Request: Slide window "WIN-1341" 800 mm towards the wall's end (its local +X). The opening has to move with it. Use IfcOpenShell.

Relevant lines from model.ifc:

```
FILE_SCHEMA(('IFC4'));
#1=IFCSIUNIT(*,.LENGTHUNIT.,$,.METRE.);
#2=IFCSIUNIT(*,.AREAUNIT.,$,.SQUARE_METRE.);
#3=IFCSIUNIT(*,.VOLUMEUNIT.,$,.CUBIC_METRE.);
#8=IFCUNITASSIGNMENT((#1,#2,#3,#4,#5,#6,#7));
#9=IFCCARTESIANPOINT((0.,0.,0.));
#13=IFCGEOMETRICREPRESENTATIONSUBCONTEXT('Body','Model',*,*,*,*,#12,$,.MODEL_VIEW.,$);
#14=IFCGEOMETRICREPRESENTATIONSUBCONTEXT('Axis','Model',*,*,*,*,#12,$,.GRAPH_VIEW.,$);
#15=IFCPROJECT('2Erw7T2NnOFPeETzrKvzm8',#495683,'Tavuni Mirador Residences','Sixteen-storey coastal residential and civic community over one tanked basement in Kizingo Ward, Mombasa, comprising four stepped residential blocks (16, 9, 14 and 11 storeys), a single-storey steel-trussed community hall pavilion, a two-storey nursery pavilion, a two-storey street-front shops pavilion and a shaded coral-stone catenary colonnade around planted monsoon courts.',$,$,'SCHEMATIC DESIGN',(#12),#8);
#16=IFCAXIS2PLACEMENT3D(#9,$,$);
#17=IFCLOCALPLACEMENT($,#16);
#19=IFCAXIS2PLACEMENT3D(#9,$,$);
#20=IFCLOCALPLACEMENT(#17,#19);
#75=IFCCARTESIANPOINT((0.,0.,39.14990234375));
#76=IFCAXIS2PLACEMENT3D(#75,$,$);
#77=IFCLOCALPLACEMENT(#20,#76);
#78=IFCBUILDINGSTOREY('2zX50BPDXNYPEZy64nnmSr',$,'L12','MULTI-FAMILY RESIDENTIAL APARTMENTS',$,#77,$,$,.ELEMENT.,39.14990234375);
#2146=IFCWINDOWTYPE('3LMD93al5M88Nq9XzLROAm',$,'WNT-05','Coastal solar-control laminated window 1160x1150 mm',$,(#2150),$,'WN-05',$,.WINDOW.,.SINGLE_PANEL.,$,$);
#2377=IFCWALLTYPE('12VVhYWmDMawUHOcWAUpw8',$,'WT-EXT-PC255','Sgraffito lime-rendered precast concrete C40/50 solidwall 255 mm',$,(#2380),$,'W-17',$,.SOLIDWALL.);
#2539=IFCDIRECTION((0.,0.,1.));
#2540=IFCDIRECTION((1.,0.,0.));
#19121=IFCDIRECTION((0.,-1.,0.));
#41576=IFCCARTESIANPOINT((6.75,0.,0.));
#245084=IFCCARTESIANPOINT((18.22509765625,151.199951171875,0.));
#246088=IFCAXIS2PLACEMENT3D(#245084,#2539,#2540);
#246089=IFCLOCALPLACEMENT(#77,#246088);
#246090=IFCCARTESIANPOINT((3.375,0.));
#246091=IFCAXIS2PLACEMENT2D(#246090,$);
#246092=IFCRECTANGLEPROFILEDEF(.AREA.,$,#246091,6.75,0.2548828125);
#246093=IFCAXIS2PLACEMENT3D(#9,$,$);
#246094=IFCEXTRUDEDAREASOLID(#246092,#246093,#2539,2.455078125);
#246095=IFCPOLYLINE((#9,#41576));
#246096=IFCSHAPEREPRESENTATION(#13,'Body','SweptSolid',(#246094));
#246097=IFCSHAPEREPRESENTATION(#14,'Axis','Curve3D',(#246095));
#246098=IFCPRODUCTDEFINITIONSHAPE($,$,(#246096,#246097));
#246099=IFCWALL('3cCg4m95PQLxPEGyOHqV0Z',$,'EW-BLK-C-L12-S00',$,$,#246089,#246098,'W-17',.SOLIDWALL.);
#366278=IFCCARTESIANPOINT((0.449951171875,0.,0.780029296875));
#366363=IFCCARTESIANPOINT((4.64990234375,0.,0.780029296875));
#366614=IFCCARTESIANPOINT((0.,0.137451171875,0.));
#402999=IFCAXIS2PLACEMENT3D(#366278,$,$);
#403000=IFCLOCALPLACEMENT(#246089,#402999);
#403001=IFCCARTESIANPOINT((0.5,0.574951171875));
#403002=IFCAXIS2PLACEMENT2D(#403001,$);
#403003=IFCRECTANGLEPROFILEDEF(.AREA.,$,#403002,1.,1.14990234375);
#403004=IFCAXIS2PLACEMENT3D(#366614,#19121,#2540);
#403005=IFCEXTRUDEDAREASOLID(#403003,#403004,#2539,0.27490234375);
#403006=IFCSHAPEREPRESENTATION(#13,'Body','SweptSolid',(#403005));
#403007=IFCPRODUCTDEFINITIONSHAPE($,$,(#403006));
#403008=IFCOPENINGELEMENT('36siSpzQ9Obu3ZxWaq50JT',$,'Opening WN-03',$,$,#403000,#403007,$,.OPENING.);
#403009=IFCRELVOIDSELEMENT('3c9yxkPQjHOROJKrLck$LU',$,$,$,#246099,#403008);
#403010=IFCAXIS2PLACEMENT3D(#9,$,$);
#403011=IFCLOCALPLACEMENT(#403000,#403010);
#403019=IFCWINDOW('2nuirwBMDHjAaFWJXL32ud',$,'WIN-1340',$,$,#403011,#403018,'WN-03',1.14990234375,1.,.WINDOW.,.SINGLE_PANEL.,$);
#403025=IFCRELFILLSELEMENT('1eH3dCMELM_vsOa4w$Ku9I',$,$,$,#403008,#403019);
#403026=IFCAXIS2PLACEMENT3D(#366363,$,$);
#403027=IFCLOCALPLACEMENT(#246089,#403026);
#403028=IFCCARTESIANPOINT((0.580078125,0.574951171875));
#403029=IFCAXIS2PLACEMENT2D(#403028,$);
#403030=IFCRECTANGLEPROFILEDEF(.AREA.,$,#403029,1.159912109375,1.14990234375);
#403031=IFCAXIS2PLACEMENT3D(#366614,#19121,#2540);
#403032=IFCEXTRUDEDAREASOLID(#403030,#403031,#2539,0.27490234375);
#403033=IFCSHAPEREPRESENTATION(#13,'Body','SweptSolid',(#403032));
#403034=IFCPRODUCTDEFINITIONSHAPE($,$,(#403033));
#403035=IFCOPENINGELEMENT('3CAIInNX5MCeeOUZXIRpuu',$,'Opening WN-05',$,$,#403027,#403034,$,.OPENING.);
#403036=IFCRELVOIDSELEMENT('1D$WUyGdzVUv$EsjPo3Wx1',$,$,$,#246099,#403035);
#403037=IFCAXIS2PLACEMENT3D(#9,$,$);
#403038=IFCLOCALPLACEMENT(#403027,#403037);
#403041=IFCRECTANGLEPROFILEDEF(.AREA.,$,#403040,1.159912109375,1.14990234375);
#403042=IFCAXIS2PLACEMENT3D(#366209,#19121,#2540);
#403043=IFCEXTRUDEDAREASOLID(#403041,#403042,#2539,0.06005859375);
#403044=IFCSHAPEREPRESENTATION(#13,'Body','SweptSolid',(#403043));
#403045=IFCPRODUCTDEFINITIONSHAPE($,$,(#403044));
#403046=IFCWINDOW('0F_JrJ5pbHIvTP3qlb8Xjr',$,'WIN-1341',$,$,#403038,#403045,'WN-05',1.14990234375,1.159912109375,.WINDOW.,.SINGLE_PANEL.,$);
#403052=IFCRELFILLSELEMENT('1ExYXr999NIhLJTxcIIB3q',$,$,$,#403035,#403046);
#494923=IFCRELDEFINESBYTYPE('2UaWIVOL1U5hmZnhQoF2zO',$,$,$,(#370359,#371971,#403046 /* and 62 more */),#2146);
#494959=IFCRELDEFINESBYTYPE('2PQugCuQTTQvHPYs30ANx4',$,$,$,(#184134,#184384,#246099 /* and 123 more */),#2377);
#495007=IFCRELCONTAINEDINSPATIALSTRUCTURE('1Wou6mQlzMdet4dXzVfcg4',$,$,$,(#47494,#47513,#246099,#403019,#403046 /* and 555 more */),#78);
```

```python
import ifcopenshell
import ifcopenshell.api.geometry
import ifcopenshell.util.placement

model = ifcopenshell.open("model.ifc")

window = model.by_guid("0F_JrJ5pbHIvTP3qlb8Xjr")
opening = window.FillsVoids[0].RelatingOpeningElement
wall = opening.VoidsElements[0].RelatingBuildingElement

wall_matrix = ifcopenshell.util.placement.get_local_placement(wall.ObjectPlacement)
shift = wall_matrix[:3, 0] * 0.8
before = ifcopenshell.util.placement.get_local_placement(window.ObjectPlacement)[:3, 3].copy()

# The window is placed relative to its opening, so it follows when the opening moves.
matrix = ifcopenshell.util.placement.get_local_placement(opening.ObjectPlacement)
matrix[:3, 3] += shift
ifcopenshell.api.geometry.edit_object_placement(
    model, product=opening, matrix=matrix, is_si=False, should_transform_children=True
)

after = ifcopenshell.util.placement.get_local_placement(window.ObjectPlacement)[:3, 3]
print("window moved by", (after - before).round(3) + 0.0)

model.write("model_updated.ifc")
```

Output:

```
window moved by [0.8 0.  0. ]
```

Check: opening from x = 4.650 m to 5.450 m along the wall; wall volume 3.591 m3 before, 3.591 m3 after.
